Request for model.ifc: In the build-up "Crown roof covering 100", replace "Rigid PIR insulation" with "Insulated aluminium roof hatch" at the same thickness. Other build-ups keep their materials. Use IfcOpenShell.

First a look at what the model holds.

```python
import ifcopenshell
import ifcopenshell.util.element

model = ifcopenshell.open("model.ifc")
print(model.schema)
for layer_set in model.by_type("IfcMaterialLayerSet"):
    if layer_set.LayerSetName == "Crown roof covering 100":
        for layer in layer_set.MaterialLayers:
            print(layer.id(), layer.Material and layer.Material.Name, layer.LayerThickness, sep=" | ")
        print(len(ifcopenshell.util.element.get_elements_by_material(model, layer_set)), "elements and types use it")
print(sorted(m.Name for m in model.by_type("IfcMaterial") if m.Name)[:60])
```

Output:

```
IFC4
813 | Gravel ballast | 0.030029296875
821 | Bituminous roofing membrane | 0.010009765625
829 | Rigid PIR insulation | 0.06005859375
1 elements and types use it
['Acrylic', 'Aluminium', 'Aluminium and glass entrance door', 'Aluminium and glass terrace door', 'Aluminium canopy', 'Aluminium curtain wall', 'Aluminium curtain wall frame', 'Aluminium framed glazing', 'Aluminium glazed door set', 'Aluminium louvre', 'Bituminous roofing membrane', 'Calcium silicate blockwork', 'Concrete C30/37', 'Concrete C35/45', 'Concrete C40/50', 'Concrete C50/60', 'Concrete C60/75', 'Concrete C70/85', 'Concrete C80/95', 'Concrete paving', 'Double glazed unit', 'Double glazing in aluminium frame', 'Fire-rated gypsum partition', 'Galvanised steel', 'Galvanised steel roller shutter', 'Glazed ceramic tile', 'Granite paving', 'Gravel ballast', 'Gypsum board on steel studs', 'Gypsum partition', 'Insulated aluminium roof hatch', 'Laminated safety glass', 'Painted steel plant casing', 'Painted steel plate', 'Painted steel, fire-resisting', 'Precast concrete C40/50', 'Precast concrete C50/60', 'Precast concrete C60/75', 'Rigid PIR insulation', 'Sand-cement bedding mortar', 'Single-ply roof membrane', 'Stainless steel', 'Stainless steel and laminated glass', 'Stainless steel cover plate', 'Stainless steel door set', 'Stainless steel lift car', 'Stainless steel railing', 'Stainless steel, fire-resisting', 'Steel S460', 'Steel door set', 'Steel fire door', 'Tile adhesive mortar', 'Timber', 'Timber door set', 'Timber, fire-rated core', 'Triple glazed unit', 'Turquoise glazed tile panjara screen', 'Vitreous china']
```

```python
import ifcopenshell
import ifcopenshell.api.material

model = ifcopenshell.open("model.ifc")

layer_set = next(s for s in model.by_type("IfcMaterialLayerSet") if s.LayerSetName == "Crown roof covering 100")
layer = next(l for l in layer_set.MaterialLayers if l.Material and l.Material.Name == "Rigid PIR insulation")
material = next(m for m in model.by_type("IfcMaterial") if m.Name == "Insulated aluminium roof hatch")

# Point this one layer at the other material; renaming the old one would change it everywhere.
ifcopenshell.api.material.edit_layer(model, layer=layer, attributes={}, material=material)

print([l.Material.Name if l.Material else None for l in layer_set.MaterialLayers])

model.write("model_edited.ifc")
```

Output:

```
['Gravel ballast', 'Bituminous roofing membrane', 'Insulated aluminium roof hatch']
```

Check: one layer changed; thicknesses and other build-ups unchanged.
